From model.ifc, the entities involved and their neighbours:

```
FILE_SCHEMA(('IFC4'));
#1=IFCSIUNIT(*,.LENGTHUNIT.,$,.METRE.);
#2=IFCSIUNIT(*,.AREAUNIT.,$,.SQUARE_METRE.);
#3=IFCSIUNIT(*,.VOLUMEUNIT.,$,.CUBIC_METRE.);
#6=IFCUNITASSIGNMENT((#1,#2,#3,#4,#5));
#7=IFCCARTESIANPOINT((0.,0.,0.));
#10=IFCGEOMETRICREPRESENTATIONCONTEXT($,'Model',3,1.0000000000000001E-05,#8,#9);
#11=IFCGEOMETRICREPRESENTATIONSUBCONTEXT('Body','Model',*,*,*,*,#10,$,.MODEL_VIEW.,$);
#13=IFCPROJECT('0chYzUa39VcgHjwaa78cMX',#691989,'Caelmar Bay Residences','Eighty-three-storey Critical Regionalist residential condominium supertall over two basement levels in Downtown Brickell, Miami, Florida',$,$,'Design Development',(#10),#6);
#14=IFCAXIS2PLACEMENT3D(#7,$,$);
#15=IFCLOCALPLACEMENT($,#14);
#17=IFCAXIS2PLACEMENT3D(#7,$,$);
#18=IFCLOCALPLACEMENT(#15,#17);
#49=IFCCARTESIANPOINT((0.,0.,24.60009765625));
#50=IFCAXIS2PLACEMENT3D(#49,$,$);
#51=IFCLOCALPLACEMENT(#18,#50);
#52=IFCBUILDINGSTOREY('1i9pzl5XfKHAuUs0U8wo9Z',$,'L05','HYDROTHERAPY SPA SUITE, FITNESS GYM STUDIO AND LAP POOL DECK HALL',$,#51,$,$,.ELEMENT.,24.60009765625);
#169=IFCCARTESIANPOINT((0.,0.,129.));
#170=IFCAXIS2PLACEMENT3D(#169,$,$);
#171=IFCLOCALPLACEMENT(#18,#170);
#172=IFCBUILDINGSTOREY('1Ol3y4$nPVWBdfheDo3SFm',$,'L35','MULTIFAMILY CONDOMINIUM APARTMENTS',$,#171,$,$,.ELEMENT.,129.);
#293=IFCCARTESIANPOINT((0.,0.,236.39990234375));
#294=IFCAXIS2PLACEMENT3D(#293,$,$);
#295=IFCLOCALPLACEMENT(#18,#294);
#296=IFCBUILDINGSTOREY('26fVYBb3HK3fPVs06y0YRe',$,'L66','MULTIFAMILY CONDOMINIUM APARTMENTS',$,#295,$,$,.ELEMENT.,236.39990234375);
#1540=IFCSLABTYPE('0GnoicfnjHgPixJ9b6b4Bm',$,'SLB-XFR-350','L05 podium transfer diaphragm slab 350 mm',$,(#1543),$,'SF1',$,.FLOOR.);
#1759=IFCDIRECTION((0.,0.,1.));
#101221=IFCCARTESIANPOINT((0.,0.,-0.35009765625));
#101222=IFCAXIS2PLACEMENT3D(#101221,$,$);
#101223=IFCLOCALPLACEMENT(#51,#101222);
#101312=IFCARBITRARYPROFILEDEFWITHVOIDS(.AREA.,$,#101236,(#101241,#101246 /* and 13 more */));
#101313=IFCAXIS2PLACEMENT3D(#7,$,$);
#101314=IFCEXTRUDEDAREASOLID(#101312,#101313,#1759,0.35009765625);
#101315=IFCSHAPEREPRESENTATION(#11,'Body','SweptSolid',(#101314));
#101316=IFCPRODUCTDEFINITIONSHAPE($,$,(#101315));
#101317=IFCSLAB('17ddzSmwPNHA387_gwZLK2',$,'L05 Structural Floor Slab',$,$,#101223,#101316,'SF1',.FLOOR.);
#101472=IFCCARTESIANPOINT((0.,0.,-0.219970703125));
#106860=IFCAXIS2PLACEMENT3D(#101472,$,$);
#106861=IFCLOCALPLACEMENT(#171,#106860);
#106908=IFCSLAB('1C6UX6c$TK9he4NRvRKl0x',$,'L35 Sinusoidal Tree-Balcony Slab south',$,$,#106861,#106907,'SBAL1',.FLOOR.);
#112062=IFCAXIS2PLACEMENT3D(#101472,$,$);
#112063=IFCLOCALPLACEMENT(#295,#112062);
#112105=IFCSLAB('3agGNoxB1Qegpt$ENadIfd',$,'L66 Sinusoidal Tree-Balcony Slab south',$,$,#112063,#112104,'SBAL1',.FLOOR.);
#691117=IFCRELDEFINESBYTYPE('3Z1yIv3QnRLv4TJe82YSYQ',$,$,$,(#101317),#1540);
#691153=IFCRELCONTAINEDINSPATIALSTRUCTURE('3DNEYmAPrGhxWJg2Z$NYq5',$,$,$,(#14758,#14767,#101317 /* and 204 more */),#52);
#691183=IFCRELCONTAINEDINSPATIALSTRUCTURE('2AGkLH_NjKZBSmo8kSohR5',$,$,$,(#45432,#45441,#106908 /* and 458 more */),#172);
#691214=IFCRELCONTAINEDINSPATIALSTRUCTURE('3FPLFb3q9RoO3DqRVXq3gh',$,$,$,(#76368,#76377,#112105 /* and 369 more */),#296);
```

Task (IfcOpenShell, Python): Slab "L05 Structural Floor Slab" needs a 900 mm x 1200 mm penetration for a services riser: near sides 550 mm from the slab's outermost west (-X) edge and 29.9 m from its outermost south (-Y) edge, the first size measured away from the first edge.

```python
import numpy as np
import ifcopenshell
import ifcopenshell.api.feature
import ifcopenshell.api.geometry
import ifcopenshell.api.root
import ifcopenshell.geom
import ifcopenshell.util.placement
import ifcopenshell.util.representation
import ifcopenshell.util.shape
import ifcopenshell.util.unit

model = ifcopenshell.open("model.ifc")
unit_scale = ifcopenshell.util.unit.calculate_unit_scale(model)
settings = ifcopenshell.geom.settings()


def volume(element):
    """Net volume in cubic metres, openings subtracted."""
    shape = ifcopenshell.geom.create_shape(settings, element)
    return ifcopenshell.util.shape.get_volume(shape.geometry)


slab = model.by_guid("17ddzSmwPNHA387_gwZLK2")
before = volume(slab)

# Extent in the slab's own axes, in metres. The edges named are its -X and -Y sides.
slab_shape = ifcopenshell.geom.create_shape(settings, slab)
vertices = ifcopenshell.util.shape.get_vertices(slab_shape.geometry)
x_min, y_min, bottom = vertices.min(axis=0)
top = vertices[:, 2].max()

opening = ifcopenshell.api.root.create_entity(model, ifc_class="IfcOpeningElement", name="Services riser opening", predefined_type="OPENING")
context = ifcopenshell.util.representation.get_context(model, "Model", "Body", "MODEL_VIEW")
width, depth = 0.9, 1.2
outline = [(0.0, 0.0), (width, 0.0), (width, depth), (0.0, depth), (0.0, 0.0)]
# Overshoot both faces by 50 mm so the cut is clean.
shape = ifcopenshell.api.geometry.add_slab_representation(
    model, context=context, depth=top - bottom + 0.1, polyline=outline
)
ifcopenshell.api.geometry.assign_representation(model, product=opening, representation=shape)

matrix = ifcopenshell.util.placement.get_local_placement(slab.ObjectPlacement)
matrix[:, 3] = matrix @ np.append(np.array([x_min + 0.55, y_min + 29.9, bottom - 0.05]) / unit_scale, 1.0)
ifcopenshell.api.geometry.edit_object_placement(model, product=opening, matrix=matrix, is_si=False)
ifcopenshell.api.feature.add_feature(model, feature=opening, element=slab)

after = volume(slab)

print(f"slab volume {before:.3f} -> {after:.3f} m3")

model.write("model_v2.ifc")
```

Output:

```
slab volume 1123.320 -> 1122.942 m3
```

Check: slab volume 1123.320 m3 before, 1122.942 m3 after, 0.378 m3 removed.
